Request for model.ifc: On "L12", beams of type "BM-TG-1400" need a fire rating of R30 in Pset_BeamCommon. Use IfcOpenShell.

First a look at what the model holds.

```python
import ifcopenshell
import ifcopenshell.util.element

model = ifcopenshell.open("model.ifc")
print(model.schema)
storey = next(s for s in model.by_type("IfcBuildingStorey") if s.Name == "L12")
beams = [e for e in ifcopenshell.util.element.get_decomposition(storey) if e.is_a("IfcBeam")]
seen = {}
for e in beams:
    element_type = ifcopenshell.util.element.get_type(e)
    key = (element_type.Name if element_type != e and element_type else None, ifcopenshell.util.element.get_pset(e, "Pset_BeamCommon", "FireRating"))
    seen[key] = seen.get(key, 0) + 1
for (name, value), count in sorted(seen.items(), key=str):
    print(count, "x", name, "|", value)
```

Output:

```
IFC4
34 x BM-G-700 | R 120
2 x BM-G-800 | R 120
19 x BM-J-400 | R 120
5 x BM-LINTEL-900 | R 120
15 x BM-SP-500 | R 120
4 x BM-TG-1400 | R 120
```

```python
import ifcopenshell
import ifcopenshell.api.pset
import ifcopenshell.util.element

model = ifcopenshell.open("model.ifc")

storey = next(s for s in model.by_type("IfcBuildingStorey") if s.Name == "L12")
beams = [e for e in ifcopenshell.util.element.get_decomposition(storey) if e.is_a("IfcBeam")]

count = 0
for e in beams:
    element_type = ifcopenshell.util.element.get_type(e)
    if element_type in (None, e) or element_type.Name != "BM-TG-1400":
        continue
    found = ifcopenshell.util.element.get_pset(e, "Pset_BeamCommon", should_inherit=False)
    if found:
        pset = model.by_id(found["id"])
        if len(ifcopenshell.util.element.get_elements_by_pset(pset)) > 1:
            pset = ifcopenshell.api.pset.unshare_pset(model, products=[e], pset=pset)[0]
    else:
        pset = ifcopenshell.api.pset.add_pset(model, product=e, name="Pset_BeamCommon")
    ifcopenshell.api.pset.edit_pset(model, pset=pset, properties={"FireRating": "R30"})
    count += 1

print(count, "beams updated")

model.write("model_v2.ifc")
```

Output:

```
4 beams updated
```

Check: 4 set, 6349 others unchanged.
